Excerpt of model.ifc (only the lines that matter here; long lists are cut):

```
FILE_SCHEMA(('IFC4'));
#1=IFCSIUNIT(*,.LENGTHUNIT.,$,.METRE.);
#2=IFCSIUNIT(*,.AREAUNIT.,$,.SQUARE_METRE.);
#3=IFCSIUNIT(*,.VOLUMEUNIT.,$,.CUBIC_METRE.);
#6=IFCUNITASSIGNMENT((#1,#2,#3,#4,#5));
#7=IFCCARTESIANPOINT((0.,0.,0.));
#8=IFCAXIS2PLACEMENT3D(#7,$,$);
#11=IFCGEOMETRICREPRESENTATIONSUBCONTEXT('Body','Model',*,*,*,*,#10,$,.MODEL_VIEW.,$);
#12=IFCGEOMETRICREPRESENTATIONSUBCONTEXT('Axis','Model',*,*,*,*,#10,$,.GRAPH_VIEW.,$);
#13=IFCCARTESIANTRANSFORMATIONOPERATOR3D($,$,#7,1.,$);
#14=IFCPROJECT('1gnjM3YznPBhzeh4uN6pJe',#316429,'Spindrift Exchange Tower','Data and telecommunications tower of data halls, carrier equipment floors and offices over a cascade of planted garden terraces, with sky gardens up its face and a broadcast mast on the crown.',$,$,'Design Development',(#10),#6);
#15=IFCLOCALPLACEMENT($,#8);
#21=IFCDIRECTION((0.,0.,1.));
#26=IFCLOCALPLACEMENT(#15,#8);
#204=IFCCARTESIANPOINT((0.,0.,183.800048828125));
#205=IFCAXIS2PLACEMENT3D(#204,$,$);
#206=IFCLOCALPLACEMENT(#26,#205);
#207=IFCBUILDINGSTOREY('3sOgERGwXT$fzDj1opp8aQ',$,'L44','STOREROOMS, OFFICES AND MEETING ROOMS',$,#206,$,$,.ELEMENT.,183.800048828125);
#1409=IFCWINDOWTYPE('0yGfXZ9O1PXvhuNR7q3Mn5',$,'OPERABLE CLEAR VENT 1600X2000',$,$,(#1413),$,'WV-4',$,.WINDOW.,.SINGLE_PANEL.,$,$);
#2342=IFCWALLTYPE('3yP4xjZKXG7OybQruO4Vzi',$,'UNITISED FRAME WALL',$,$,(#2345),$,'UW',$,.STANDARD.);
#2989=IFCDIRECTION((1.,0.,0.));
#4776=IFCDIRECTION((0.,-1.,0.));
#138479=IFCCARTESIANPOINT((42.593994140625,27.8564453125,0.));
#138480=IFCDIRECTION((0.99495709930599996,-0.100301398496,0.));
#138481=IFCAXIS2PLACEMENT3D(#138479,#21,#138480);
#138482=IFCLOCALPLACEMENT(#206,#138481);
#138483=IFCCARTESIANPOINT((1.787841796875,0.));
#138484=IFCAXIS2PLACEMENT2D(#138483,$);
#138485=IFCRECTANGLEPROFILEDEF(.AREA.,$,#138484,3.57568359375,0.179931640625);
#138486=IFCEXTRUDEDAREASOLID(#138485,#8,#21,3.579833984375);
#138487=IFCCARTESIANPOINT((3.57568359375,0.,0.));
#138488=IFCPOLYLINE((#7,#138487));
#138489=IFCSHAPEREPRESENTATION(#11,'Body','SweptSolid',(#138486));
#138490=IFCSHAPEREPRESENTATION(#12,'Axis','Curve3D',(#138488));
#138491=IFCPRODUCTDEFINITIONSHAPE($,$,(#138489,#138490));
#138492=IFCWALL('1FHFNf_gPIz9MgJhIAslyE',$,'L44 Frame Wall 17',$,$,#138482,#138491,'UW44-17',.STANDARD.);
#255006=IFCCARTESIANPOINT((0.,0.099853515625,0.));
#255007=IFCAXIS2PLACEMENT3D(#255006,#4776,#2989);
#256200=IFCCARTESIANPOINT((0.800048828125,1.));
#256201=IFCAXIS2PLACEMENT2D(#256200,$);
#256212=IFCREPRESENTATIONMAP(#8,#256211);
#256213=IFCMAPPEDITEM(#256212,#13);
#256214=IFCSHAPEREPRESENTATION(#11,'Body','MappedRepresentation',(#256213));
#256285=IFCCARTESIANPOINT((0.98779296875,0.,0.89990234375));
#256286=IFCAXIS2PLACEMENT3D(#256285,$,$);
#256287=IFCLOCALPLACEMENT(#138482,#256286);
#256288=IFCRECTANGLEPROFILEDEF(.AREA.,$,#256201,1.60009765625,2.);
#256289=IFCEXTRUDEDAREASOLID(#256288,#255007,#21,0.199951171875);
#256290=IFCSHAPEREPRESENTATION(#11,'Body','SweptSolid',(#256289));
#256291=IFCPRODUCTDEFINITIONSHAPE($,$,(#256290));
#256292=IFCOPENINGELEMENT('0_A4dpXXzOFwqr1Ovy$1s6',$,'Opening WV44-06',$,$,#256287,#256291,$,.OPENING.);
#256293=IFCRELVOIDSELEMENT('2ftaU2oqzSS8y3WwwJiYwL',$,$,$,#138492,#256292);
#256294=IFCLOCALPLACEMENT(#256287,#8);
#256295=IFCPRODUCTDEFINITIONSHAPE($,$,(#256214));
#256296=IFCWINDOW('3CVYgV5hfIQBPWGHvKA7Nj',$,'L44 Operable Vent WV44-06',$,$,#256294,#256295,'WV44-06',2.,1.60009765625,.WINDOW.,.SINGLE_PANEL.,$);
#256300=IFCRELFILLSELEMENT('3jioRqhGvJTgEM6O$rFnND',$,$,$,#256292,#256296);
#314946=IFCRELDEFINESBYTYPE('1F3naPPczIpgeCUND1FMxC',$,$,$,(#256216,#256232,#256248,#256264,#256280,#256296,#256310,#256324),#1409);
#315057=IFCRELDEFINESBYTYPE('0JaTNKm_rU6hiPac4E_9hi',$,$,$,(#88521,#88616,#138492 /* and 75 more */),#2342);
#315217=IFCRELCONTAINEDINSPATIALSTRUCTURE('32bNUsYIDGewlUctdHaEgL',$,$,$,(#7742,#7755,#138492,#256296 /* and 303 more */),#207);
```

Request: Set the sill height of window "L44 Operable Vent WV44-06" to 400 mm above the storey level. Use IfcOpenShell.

```python
import numpy as np
import ifcopenshell
import ifcopenshell.api.geometry
import ifcopenshell.geom
import ifcopenshell.util.element
import ifcopenshell.util.placement
import ifcopenshell.util.shape
import ifcopenshell.util.unit

model = ifcopenshell.open("model.ifc")
unit_scale = ifcopenshell.util.unit.calculate_unit_scale(model)

window = model.by_guid("3CVYgV5hfIQBPWGHvKA7Nj")
opening = window.FillsVoids[0].RelatingOpeningElement
storey = ifcopenshell.util.element.get_container(window, ifc_class="IfcBuildingStorey")
level = ifcopenshell.util.placement.get_local_placement(storey.ObjectPlacement)[2, 3]

# The opening's origin need not be at the sill, so measure its lowest point.
shape = ifcopenshell.geom.create_shape(ifcopenshell.geom.settings(), opening)
bottom = ifcopenshell.util.shape.get_shape_bottom_elevation(shape, shape.geometry) / unit_scale
dz = level + 0.4 / unit_scale - bottom

shift = np.array([0.0, 0.0, dz])
# The window is placed relative to its opening, so it follows when the opening moves.
matrix = ifcopenshell.util.placement.get_local_placement(opening.ObjectPlacement)
matrix[:3, 3] += shift
ifcopenshell.api.geometry.edit_object_placement(
    model, product=opening, matrix=matrix, is_si=False, should_transform_children=True
)

print(f"moved by {dz * unit_scale:+.3f} m")

model.write("model-out.ifc")
```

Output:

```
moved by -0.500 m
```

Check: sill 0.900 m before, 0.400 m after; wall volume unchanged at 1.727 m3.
